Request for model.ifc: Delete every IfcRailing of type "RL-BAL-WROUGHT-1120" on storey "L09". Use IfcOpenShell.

First a look at what the model holds.

```python
import ifcopenshell
import ifcopenshell.util.element

model = ifcopenshell.open("model.ifc")
print(model.schema)
storey = next(s for s in model.by_type("IfcBuildingStorey") if s.Name == "L09")
railings = [e for e in ifcopenshell.util.element.get_decomposition(storey) if e.is_a("IfcRailing")]
seen = {}
for e in railings:
    element_type = ifcopenshell.util.element.get_type(e)
    name = element_type.Name if element_type not in (None, e) else None
    seen[name] = seen.get(name, 0) + 1
for name, count in sorted(seen.items(), key=str):
    print(count, "x", name)
```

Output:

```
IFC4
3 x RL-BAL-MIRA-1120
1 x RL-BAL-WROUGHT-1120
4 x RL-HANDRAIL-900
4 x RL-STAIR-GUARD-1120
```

```python
import ifcopenshell
import ifcopenshell.api.root
import ifcopenshell.util.element

model = ifcopenshell.open("model.ifc")

storey = next(s for s in model.by_type("IfcBuildingStorey") if s.Name == "L09")
railings = [e for e in ifcopenshell.util.element.get_decomposition(storey) if e.is_a("IfcRailing")]
targets = [e for e in railings if (t := ifcopenshell.util.element.get_type(e)) not in (None, e) and t.Name == "RL-BAL-WROUGHT-1120"]

for e in targets:
    ifcopenshell.api.root.remove_product(model, product=e)
print(len(targets), "removed")

model.write("model_edited.ifc")
```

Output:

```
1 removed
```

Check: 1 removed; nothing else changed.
